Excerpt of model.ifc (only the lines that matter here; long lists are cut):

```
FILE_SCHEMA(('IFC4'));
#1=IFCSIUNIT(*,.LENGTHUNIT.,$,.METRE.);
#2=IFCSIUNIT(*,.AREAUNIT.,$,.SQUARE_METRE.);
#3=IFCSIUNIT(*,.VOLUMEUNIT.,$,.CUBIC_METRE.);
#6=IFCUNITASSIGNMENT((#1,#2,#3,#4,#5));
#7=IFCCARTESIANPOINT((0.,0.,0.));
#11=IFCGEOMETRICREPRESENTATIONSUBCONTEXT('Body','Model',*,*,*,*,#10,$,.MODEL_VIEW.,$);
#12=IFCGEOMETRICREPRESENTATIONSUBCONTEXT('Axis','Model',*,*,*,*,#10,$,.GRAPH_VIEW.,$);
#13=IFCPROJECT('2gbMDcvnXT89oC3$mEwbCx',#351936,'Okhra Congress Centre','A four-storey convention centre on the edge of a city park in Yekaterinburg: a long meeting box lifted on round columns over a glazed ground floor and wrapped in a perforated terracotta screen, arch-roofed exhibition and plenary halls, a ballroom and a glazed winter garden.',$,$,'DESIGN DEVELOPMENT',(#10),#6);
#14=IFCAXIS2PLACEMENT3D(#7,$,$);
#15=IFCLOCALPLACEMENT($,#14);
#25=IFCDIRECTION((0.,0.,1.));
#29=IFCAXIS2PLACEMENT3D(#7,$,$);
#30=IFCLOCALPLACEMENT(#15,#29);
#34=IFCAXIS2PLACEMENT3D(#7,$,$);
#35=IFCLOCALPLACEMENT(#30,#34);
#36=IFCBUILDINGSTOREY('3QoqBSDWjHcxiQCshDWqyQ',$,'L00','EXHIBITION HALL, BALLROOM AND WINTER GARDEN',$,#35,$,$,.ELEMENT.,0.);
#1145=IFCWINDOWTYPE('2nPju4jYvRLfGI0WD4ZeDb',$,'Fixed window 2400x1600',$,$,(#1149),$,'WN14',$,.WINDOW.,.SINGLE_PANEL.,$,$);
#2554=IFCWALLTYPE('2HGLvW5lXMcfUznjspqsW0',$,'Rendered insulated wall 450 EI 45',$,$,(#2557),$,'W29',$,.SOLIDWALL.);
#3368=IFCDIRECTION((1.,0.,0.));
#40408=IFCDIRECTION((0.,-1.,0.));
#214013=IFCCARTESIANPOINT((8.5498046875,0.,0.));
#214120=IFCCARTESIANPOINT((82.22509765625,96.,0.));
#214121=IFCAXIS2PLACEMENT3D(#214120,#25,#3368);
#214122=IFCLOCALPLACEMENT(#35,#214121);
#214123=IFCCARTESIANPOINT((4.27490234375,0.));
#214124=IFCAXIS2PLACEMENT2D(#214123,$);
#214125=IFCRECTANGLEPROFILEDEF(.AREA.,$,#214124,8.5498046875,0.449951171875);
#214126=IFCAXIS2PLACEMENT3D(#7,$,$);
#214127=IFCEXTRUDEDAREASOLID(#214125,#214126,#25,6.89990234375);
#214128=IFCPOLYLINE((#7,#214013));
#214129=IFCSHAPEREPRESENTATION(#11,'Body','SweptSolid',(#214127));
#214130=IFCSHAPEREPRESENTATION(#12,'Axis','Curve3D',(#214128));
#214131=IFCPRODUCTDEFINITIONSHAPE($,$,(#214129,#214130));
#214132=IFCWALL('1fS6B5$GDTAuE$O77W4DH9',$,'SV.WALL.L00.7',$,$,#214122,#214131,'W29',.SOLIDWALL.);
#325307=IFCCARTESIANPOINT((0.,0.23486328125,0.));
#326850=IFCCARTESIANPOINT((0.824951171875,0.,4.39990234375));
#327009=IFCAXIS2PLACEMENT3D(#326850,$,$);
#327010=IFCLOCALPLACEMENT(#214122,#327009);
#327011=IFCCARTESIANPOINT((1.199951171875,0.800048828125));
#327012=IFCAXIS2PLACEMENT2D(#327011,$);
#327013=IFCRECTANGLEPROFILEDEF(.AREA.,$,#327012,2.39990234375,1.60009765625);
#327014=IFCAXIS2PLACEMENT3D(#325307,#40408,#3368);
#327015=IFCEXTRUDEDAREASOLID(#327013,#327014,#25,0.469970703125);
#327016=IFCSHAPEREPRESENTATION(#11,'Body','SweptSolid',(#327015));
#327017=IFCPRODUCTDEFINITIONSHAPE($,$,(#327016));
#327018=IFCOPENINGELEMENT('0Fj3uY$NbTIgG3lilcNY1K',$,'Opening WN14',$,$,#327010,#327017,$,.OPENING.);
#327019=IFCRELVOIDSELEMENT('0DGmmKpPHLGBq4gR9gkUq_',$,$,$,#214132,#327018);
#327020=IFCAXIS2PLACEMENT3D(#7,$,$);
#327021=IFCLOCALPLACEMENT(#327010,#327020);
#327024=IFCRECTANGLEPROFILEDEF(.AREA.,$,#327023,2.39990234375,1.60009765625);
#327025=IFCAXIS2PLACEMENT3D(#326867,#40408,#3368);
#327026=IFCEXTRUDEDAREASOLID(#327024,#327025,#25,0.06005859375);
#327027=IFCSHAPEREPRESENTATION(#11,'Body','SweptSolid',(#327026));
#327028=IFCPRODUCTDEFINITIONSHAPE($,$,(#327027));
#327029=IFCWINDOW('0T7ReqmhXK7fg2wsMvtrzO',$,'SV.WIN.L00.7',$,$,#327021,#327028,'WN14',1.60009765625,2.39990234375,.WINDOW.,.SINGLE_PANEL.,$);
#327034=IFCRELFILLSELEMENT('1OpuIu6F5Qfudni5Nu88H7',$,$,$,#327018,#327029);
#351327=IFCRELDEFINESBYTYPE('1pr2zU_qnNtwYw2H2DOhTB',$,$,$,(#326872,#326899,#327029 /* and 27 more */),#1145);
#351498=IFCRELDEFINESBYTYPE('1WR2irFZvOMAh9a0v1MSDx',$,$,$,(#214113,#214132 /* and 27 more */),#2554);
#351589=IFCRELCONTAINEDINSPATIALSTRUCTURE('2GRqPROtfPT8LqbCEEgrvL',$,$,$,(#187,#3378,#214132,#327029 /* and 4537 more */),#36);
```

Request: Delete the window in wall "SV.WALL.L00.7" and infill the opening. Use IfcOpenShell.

```python
import ifcopenshell
import ifcopenshell.api.feature
import ifcopenshell.api.root
import ifcopenshell.geom
import ifcopenshell.util.shape

model = ifcopenshell.open("model.ifc")
settings = ifcopenshell.geom.settings()


def volume(element):
    """Net volume in cubic metres, openings subtracted."""
    shape = ifcopenshell.geom.create_shape(settings, element)
    return ifcopenshell.util.shape.get_volume(shape.geometry)


window = model.by_guid("0T7ReqmhXK7fg2wsMvtrzO")
opening = window.FillsVoids[0].RelatingOpeningElement
wall = opening.VoidsElements[0].RelatingBuildingElement
before = volume(wall)

ifcopenshell.api.root.remove_product(model, product=window)
ifcopenshell.api.feature.remove_feature(model, feature=opening)

after = volume(wall)

print(f"wall volume {before:.3f} -> {after:.3f} m3")

model.write("model-out.ifc")
```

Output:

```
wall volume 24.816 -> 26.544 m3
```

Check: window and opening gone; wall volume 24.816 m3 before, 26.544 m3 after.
